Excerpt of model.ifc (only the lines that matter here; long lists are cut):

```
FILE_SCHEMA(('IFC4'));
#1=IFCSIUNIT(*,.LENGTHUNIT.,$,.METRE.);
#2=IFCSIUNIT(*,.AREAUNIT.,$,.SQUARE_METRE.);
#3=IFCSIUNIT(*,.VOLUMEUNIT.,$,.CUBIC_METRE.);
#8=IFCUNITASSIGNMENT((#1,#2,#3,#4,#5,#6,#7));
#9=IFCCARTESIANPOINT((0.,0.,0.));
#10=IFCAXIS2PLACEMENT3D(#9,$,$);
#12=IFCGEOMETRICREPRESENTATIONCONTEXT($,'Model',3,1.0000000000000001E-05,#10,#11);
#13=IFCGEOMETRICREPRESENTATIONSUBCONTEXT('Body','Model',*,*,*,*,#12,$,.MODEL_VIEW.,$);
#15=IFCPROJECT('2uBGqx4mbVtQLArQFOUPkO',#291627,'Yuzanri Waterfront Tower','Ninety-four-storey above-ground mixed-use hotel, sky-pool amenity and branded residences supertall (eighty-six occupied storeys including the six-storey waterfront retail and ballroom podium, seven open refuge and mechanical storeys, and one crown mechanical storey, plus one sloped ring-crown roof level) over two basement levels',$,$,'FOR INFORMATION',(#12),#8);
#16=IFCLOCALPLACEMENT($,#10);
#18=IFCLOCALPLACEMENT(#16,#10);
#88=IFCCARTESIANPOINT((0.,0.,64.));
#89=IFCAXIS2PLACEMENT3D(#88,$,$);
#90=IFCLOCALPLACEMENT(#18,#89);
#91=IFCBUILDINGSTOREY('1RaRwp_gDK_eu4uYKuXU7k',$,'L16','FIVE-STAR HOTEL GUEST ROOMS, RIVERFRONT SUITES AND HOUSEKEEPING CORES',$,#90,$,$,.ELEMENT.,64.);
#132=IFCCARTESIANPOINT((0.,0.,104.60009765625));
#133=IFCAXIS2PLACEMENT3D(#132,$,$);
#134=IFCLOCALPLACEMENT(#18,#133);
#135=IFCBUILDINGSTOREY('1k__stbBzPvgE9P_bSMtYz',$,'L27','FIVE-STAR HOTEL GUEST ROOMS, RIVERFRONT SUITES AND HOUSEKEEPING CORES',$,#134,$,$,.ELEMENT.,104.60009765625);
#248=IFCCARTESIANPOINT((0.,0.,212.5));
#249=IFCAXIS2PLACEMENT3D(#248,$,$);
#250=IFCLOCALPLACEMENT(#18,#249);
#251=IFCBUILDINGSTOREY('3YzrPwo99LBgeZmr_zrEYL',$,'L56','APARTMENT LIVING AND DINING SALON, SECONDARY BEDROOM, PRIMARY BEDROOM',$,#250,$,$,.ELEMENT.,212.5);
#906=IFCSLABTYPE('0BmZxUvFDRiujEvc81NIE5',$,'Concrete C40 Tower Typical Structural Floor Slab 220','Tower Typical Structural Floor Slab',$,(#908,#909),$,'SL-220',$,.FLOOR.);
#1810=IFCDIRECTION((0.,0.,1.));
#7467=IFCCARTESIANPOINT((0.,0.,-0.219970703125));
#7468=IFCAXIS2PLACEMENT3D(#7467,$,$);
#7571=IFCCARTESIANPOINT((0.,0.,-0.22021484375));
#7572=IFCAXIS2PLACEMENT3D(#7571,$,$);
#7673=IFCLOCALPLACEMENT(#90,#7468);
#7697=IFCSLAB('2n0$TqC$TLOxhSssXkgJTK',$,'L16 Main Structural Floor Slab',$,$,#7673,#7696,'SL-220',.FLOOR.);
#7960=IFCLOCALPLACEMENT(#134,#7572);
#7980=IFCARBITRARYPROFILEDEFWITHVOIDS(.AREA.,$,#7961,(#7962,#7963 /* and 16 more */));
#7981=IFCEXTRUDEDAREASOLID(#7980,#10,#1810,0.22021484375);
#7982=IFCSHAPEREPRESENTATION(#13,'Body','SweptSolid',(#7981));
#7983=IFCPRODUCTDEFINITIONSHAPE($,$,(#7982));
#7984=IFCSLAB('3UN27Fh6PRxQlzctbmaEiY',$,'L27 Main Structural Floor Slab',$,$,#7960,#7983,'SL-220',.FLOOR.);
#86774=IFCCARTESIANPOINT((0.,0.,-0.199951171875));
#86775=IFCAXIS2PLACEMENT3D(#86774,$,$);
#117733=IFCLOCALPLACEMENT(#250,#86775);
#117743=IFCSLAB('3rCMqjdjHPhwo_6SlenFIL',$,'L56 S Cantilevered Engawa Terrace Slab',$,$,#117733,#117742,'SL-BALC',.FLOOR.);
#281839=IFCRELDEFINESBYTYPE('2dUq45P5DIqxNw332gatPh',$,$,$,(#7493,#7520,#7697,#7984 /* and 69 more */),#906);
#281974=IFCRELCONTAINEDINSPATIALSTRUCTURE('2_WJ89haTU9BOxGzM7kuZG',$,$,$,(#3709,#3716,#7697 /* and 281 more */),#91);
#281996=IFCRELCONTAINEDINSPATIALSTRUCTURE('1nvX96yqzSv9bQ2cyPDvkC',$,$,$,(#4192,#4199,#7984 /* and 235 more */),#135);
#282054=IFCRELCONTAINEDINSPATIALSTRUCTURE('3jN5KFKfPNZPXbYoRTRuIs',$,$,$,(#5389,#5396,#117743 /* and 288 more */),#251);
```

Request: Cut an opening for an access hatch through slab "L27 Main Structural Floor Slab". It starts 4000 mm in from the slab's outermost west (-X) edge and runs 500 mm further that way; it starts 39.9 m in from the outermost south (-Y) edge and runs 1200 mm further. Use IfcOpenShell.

```python
import numpy as np
import ifcopenshell
import ifcopenshell.api.feature
import ifcopenshell.api.geometry
import ifcopenshell.api.root
import ifcopenshell.geom
import ifcopenshell.util.placement
import ifcopenshell.util.representation
import ifcopenshell.util.shape
import ifcopenshell.util.unit

model = ifcopenshell.open("model.ifc")
unit_scale = ifcopenshell.util.unit.calculate_unit_scale(model)
settings = ifcopenshell.geom.settings()


def volume(element):
    """Net volume in cubic metres, openings subtracted."""
    shape = ifcopenshell.geom.create_shape(settings, element)
    return ifcopenshell.util.shape.get_volume(shape.geometry)


slab = model.by_guid("3UN27Fh6PRxQlzctbmaEiY")
before = volume(slab)

# Extent in the slab's own axes, in metres. The edges named are its -X and -Y sides.
slab_shape = ifcopenshell.geom.create_shape(settings, slab)
vertices = ifcopenshell.util.shape.get_vertices(slab_shape.geometry)
x_min, y_min, bottom = vertices.min(axis=0)
top = vertices[:, 2].max()

opening = ifcopenshell.api.root.create_entity(model, ifc_class="IfcOpeningElement", name="Access hatch opening", predefined_type="OPENING")
context = ifcopenshell.util.representation.get_context(model, "Model", "Body", "MODEL_VIEW")
width, depth = 0.5, 1.2
outline = [(0.0, 0.0), (width, 0.0), (width, depth), (0.0, depth), (0.0, 0.0)]
# Overshoot both faces by 50 mm so the cut is clean.
shape = ifcopenshell.api.geometry.add_slab_representation(
    model, context=context, depth=top - bottom + 0.1, polyline=outline
)
ifcopenshell.api.geometry.assign_representation(model, product=opening, representation=shape)

matrix = ifcopenshell.util.placement.get_local_placement(slab.ObjectPlacement)
matrix[:, 3] = matrix @ np.append(np.array([x_min + 4, y_min + 39.9, bottom - 0.05]) / unit_scale, 1.0)
ifcopenshell.api.geometry.edit_object_placement(model, product=opening, matrix=matrix, is_si=False)
ifcopenshell.api.feature.add_feature(model, feature=opening, element=slab)

after = volume(slab)

print(f"slab volume {before:.3f} -> {after:.3f} m3")

model.write("model_edited.ifc")
```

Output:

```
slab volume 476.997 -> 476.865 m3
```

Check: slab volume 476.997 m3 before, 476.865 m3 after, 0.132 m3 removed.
